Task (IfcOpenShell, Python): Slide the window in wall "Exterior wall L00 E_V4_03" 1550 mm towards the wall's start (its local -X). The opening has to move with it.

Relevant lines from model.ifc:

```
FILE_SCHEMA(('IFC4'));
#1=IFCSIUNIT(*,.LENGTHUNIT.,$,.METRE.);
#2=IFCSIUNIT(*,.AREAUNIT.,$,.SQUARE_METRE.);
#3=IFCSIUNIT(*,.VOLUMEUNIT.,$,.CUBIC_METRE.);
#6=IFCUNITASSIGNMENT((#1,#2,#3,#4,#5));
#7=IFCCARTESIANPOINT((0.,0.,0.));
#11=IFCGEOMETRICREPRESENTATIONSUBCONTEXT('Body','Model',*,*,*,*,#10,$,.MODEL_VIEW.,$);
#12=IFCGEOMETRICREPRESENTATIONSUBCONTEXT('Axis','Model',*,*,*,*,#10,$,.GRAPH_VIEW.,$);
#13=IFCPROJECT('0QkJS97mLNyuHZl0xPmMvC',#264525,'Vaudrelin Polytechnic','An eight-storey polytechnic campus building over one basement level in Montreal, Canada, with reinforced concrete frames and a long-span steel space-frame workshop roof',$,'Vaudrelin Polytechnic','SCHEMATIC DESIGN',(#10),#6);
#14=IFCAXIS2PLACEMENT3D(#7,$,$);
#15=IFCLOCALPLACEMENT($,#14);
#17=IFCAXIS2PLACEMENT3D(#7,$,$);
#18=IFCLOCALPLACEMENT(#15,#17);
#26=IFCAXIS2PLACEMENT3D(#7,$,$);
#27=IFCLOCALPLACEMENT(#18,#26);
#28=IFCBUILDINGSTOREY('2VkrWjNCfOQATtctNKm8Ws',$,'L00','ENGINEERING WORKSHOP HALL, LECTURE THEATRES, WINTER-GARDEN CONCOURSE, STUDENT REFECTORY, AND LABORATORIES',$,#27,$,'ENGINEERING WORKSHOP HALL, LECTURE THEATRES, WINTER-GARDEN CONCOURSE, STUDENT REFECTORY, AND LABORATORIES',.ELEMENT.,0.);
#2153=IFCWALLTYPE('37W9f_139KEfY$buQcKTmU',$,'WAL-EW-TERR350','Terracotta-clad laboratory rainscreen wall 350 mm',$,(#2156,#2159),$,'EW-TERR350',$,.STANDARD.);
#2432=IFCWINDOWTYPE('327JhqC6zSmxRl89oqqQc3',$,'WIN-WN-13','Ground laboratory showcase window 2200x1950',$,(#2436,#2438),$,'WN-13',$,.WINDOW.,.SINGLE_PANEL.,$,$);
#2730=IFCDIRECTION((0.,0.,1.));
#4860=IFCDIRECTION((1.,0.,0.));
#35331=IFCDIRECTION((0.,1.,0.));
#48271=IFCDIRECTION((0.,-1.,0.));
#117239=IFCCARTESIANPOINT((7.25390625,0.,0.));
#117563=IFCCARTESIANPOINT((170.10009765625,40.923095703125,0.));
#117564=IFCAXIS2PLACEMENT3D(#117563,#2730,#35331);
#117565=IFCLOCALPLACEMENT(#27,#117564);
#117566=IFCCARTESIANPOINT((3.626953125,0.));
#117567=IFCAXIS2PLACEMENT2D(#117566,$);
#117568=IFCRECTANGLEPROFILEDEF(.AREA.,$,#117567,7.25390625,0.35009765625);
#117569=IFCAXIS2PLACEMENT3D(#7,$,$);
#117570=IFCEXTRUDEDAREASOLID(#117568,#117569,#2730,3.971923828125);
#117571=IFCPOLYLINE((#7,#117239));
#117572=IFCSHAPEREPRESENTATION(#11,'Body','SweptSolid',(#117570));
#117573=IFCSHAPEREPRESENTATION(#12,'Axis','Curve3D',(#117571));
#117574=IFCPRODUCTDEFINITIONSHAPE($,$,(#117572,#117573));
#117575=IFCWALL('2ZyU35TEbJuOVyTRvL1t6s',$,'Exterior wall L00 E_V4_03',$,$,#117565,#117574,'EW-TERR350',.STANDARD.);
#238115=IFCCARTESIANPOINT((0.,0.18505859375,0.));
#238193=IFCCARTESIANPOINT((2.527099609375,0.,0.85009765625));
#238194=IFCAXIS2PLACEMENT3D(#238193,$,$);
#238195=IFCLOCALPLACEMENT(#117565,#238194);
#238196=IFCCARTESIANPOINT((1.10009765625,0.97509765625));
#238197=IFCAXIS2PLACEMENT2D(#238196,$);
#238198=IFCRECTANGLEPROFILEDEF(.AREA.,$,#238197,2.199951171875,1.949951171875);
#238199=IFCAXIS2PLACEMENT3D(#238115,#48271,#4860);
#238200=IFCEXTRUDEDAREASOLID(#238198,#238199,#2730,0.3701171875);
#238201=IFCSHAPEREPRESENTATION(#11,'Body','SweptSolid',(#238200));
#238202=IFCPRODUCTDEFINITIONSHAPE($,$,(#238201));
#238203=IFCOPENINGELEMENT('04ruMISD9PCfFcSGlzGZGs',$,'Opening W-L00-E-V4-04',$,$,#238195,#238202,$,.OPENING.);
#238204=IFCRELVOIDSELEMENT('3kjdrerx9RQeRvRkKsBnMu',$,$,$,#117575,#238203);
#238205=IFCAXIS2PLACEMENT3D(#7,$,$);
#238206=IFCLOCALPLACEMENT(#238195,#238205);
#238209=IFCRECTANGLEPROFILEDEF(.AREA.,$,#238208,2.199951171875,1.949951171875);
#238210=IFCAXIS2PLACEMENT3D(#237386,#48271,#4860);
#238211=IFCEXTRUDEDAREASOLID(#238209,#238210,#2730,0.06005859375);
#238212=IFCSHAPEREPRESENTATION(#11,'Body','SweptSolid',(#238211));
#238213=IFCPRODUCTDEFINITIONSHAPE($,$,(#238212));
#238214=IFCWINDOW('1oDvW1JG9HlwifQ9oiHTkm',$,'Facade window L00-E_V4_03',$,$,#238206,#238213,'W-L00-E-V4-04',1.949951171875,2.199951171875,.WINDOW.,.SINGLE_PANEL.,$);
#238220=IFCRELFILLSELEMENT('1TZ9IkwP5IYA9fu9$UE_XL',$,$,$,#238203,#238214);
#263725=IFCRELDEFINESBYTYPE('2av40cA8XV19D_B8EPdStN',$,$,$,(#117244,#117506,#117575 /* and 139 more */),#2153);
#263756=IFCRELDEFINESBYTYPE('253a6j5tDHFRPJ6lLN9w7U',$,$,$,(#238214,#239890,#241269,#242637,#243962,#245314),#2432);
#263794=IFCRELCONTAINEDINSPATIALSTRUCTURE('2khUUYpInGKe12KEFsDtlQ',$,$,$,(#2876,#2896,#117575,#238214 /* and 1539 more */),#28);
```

```python
import ifcopenshell
import ifcopenshell.api.geometry
import ifcopenshell.util.placement
import ifcopenshell.util.unit

model = ifcopenshell.open("model.ifc")
unit_scale = ifcopenshell.util.unit.calculate_unit_scale(model)

window = model.by_guid("1oDvW1JG9HlwifQ9oiHTkm")
opening = window.FillsVoids[0].RelatingOpeningElement
wall = opening.VoidsElements[0].RelatingBuildingElement

wall_matrix = ifcopenshell.util.placement.get_local_placement(wall.ObjectPlacement)
shift = wall_matrix[:3, 0] * -1.55 / unit_scale
before = ifcopenshell.util.placement.get_local_placement(window.ObjectPlacement)[:3, 3].copy()

# The window is placed relative to its opening, so it follows when the opening moves.
matrix = ifcopenshell.util.placement.get_local_placement(opening.ObjectPlacement)
matrix[:3, 3] += shift
ifcopenshell.api.geometry.edit_object_placement(
    model, product=opening, matrix=matrix, is_si=False, should_transform_children=True
)

after = ifcopenshell.util.placement.get_local_placement(window.ObjectPlacement)[:3, 3]
print("window moved by", (after - before).round(3) + 0.0)

model.write("model_updated.ifc")
```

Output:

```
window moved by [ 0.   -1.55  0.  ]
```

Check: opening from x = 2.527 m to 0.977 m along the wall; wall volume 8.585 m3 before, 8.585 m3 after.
